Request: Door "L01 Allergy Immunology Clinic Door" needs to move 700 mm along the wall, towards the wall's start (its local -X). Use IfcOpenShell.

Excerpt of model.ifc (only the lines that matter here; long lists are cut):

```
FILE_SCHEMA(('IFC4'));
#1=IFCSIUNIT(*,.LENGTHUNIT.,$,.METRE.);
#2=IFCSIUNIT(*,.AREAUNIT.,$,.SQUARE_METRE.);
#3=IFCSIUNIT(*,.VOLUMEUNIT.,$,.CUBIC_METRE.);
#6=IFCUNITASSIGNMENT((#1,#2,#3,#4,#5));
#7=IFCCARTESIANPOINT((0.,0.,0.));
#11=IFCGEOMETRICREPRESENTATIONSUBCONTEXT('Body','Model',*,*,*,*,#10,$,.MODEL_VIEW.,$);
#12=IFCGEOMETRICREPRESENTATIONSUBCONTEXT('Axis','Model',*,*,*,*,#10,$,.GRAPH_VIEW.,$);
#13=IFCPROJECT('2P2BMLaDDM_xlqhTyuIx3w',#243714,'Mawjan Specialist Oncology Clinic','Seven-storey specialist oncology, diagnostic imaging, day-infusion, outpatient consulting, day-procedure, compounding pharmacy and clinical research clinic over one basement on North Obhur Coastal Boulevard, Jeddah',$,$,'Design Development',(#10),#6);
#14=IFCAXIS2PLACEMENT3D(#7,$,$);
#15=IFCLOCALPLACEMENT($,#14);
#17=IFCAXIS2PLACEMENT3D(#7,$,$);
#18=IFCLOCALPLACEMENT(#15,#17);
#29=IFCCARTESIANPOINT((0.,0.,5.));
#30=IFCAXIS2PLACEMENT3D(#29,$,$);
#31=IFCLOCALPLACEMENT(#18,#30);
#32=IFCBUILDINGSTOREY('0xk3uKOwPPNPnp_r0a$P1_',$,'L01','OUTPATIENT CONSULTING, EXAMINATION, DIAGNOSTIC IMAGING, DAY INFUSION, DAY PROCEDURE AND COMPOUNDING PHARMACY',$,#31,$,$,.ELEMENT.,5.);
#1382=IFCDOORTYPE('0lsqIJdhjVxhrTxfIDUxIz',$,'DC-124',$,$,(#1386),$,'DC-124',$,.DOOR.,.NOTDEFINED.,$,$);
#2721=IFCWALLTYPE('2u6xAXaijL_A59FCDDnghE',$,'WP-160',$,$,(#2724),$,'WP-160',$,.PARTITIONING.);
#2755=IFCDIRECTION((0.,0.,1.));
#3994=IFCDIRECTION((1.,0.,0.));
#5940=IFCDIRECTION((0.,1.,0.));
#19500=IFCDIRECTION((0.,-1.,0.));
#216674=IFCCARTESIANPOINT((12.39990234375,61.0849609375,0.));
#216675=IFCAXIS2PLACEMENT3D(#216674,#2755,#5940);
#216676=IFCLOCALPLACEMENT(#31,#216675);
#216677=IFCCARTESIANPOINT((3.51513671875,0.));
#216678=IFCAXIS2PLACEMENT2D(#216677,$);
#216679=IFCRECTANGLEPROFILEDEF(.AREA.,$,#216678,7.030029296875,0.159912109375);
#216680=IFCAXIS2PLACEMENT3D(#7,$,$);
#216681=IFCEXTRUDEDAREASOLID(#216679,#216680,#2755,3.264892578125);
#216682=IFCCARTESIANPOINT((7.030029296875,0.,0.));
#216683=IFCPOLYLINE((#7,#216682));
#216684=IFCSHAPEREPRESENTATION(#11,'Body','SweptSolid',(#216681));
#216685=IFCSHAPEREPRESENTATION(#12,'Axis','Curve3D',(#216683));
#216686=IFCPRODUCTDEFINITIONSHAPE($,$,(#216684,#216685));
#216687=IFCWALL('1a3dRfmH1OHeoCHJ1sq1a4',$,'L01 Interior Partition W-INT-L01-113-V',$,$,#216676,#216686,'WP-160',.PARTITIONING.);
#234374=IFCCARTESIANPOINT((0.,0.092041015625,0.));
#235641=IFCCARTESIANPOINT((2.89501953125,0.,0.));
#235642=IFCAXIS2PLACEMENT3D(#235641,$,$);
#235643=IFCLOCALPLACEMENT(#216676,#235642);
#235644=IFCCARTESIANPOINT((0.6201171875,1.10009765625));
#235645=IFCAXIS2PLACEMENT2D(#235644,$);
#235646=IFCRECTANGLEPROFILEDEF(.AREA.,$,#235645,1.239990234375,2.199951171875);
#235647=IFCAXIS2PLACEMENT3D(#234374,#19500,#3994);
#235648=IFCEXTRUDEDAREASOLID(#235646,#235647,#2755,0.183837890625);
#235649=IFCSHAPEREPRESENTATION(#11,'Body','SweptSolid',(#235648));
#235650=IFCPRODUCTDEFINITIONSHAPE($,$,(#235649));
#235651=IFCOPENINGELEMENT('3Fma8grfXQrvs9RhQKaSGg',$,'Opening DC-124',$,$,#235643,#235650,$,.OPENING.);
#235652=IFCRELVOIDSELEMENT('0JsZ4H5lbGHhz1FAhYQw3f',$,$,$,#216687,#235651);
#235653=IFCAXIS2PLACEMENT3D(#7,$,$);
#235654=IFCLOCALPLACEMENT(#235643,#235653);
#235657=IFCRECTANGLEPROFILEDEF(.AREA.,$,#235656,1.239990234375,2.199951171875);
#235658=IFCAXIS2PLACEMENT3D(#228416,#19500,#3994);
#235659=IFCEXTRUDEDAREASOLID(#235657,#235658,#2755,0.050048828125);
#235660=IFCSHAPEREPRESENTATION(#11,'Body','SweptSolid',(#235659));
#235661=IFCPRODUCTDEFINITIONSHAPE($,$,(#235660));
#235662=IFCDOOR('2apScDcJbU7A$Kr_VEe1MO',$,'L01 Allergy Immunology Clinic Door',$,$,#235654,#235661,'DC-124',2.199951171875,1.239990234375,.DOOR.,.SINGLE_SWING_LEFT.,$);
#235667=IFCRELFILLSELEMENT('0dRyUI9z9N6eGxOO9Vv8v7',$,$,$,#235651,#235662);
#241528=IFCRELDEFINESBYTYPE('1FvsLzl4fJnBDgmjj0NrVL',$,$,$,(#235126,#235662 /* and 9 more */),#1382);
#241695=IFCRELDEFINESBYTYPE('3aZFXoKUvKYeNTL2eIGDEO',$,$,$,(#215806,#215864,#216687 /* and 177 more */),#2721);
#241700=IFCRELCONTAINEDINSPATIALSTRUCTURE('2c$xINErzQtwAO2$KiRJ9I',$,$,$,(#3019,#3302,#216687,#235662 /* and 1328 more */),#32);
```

```python
import ifcopenshell
import ifcopenshell.api.geometry
import ifcopenshell.util.placement
import ifcopenshell.util.unit

model = ifcopenshell.open("model.ifc")
unit_scale = ifcopenshell.util.unit.calculate_unit_scale(model)

door = model.by_id(235662)
opening = door.FillsVoids[0].RelatingOpeningElement
wall = opening.VoidsElements[0].RelatingBuildingElement

wall_matrix = ifcopenshell.util.placement.get_local_placement(wall.ObjectPlacement)
shift = wall_matrix[:3, 0] * -0.7 / unit_scale
before = ifcopenshell.util.placement.get_local_placement(door.ObjectPlacement)[:3, 3].copy()

# The door is placed relative to its opening, so it follows when the opening moves.
matrix = ifcopenshell.util.placement.get_local_placement(opening.ObjectPlacement)
matrix[:3, 3] += shift
ifcopenshell.api.geometry.edit_object_placement(
    model, product=opening, matrix=matrix, is_si=False, should_transform_children=True
)

after = ifcopenshell.util.placement.get_local_placement(door.ObjectPlacement)[:3, 3]
print("door moved by", (after - before).round(3) + 0.0)

model.write("model_rev.ifc")
```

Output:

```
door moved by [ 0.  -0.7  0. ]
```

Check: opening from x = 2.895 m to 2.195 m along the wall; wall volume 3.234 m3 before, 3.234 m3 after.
